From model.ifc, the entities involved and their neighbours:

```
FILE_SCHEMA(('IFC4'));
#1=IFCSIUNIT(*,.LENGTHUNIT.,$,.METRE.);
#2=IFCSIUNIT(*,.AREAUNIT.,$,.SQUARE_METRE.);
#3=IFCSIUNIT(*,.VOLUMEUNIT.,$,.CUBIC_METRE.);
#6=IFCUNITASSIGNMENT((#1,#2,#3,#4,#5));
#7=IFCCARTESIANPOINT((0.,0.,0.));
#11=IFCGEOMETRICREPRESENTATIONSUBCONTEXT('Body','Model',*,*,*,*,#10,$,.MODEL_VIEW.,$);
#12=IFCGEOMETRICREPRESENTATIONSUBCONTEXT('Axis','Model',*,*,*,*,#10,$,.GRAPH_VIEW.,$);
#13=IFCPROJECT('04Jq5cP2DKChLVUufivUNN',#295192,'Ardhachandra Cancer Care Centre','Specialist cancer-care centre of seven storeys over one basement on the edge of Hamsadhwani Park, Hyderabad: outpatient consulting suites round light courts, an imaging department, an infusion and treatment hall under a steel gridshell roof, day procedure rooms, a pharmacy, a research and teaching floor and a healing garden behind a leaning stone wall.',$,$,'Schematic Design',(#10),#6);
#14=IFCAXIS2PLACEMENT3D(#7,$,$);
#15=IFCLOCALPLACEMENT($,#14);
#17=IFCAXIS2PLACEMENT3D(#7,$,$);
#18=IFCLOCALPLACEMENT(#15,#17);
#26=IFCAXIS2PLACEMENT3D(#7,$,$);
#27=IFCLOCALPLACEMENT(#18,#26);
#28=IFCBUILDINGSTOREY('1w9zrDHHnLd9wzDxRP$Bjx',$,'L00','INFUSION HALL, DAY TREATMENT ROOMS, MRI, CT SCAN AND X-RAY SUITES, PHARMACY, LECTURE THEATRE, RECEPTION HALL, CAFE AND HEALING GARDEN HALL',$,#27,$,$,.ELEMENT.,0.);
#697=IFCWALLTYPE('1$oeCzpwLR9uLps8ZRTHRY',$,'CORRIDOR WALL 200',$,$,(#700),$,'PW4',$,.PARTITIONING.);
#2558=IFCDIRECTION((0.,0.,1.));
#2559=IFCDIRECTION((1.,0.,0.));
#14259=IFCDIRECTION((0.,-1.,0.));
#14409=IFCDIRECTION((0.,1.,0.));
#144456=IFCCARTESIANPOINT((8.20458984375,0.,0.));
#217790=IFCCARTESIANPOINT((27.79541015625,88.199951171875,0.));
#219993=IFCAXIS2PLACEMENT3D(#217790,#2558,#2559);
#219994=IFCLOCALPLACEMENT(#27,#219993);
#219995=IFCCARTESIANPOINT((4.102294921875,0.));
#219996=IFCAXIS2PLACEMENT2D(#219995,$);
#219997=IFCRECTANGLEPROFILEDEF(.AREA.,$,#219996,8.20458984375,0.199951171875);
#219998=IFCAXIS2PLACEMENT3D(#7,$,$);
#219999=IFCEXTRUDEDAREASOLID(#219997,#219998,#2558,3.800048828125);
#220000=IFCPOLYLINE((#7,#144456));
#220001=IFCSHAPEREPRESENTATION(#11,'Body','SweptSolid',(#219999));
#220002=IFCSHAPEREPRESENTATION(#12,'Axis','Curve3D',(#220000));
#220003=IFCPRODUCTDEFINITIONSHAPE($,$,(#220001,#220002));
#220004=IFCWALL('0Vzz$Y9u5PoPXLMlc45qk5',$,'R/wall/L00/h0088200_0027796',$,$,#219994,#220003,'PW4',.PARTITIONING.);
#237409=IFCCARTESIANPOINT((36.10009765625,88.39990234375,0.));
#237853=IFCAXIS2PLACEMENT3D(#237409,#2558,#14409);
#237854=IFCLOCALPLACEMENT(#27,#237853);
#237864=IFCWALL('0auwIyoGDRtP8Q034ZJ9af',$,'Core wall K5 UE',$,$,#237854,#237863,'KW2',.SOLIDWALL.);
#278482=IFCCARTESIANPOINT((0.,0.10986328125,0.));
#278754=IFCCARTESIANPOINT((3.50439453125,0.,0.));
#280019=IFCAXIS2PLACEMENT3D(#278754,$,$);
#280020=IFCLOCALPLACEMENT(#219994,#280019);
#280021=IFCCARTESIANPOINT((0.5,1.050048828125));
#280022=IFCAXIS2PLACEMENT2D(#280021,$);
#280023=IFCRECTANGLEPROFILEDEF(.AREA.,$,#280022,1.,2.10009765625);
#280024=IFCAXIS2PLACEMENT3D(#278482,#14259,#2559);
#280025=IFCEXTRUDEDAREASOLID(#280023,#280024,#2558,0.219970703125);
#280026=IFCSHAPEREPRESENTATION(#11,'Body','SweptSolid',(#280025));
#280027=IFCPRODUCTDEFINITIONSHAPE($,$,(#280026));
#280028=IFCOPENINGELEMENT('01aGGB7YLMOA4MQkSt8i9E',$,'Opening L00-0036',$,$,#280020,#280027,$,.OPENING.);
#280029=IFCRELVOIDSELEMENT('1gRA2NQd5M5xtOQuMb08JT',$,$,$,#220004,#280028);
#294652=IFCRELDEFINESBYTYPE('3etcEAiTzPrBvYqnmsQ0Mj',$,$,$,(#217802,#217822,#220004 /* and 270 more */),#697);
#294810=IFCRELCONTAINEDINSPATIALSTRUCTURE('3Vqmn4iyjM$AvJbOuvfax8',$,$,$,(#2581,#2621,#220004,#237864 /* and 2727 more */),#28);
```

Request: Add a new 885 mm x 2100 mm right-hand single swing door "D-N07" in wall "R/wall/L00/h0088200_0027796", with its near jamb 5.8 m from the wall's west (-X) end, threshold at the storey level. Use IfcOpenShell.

```python
import numpy as np
import ifcopenshell
import ifcopenshell.api.feature
import ifcopenshell.api.geometry
import ifcopenshell.api.root
import ifcopenshell.api.spatial
import ifcopenshell.geom
import ifcopenshell.util.element
import ifcopenshell.util.placement
import ifcopenshell.util.representation
import ifcopenshell.util.shape
import ifcopenshell.util.unit

model = ifcopenshell.open("model.ifc")
unit_scale = ifcopenshell.util.unit.calculate_unit_scale(model)
settings = ifcopenshell.geom.settings()


def volume(element):
    """Net volume in cubic metres, openings subtracted."""
    shape = ifcopenshell.geom.create_shape(settings, element)
    return ifcopenshell.util.shape.get_volume(shape.geometry)


wall = model.by_guid("0Vzz$Y9u5PoPXLMlc45qk5")
storey = ifcopenshell.util.element.get_container(wall, ifc_class="IfcBuildingStorey")
context = ifcopenshell.util.representation.get_context(model, "Model", "Body", "MODEL_VIEW")
before = volume(wall)

width, height, from_end, sill = 0.885, 2.1, 5.8, 0.0  # metres

# The wall runs along its own X axis, and the end named is its -X end.
wall_shape = ifcopenshell.geom.create_shape(settings, wall)
x, y, z = ifcopenshell.util.shape.get_vertices(wall_shape.geometry).T
start = x.min() + from_end
face, thickness = float(y.min()), float(y.max() - y.min())
wall_matrix = ifcopenshell.util.placement.get_local_placement(wall.ObjectPlacement)
level = ifcopenshell.util.placement.get_local_placement(storey.ObjectPlacement)[2, 3]


def in_wall(x, y):
    """Placement at x, y metres in the wall's axes, at sill height."""
    matrix = wall_matrix.copy()
    matrix[:, 3] = wall_matrix @ np.array([x / unit_scale, y / unit_scale, 0.0, 1.0])
    matrix[2, 3] = level + sill / unit_scale
    return matrix


# Opening: a box that overshoots both wall faces by 50 mm.
opening = ifcopenshell.api.root.create_entity(model, ifc_class="IfcOpeningElement", predefined_type="OPENING")
box = ifcopenshell.api.geometry.add_wall_representation(
    model, context=context, length=width, height=height, thickness=thickness + 0.1
)
ifcopenshell.api.geometry.assign_representation(model, product=opening, representation=box)
ifcopenshell.api.geometry.edit_object_placement(model, product=opening, matrix=in_wall(start, face - 0.05), is_si=False)
ifcopenshell.api.feature.add_feature(model, feature=opening, element=wall)

door = ifcopenshell.api.root.create_entity(model, ifc_class="IfcDoor", name="D-N07", predefined_type="DOOR")
door.OverallWidth, door.OverallHeight = width / unit_scale, height / unit_scale
door.OperationType = "SINGLE_SWING_RIGHT"
body = ifcopenshell.api.geometry.add_door_representation(
    model,
    context=context,
    overall_width=door.OverallWidth,
    overall_height=door.OverallHeight,
    operation_type="SINGLE_SWING_RIGHT",
    lining_properties={"LiningDepth": thickness / unit_scale, "ThresholdDepth": thickness / unit_scale},
)
ifcopenshell.api.geometry.assign_representation(model, product=door, representation=body)
ifcopenshell.api.spatial.assign_container(model, products=[door], relating_structure=storey)
ifcopenshell.api.feature.add_filling(model, opening=opening, element=door)

# The lining spans the wall, so the door starts at the wall face.
ifcopenshell.api.geometry.edit_object_placement(model, product=door, matrix=in_wall(start, face), is_si=False)

after = volume(wall)

print(f"wall volume {before:.3f} -> {after:.3f} m3")

model.write("model-out.ifc")
```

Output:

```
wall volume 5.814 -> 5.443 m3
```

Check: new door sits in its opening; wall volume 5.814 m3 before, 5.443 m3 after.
